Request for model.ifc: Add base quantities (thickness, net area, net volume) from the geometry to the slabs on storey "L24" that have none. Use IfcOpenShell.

First a look at what the model holds.

```python
import ifcopenshell
import ifcopenshell.util.element
import ifcopenshell.util.unit

model = ifcopenshell.open("model.ifc")
print(model.schema)
for unit_type in ("LENGTHUNIT", "AREAUNIT", "VOLUMEUNIT"):
    print(unit_type, ifcopenshell.util.unit.calculate_unit_scale(model, unit_type))
storey = next(s for s in model.by_type("IfcBuildingStorey") if s.Name == "L24")
slabs = [e for e in ifcopenshell.util.element.get_decomposition(storey) if e.is_a("IfcSlab")]
for e in sorted(slabs, key=lambda e: e.id()):
    print(e.id(), e.is_a(), e.Name, list(ifcopenshell.util.element.get_psets(e, qtos_only=True)), sep=" | ")
```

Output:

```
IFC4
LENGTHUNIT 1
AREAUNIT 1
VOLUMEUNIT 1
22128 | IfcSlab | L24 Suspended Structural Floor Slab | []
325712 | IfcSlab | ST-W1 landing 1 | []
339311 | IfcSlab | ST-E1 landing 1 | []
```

```python
import ifcopenshell
import ifcopenshell.api.pset
import ifcopenshell.geom
import ifcopenshell.util.element
import ifcopenshell.util.shape
import ifcopenshell.util.unit

model = ifcopenshell.open("model.ifc")
unit_scale = ifcopenshell.util.unit.calculate_unit_scale(model)
area_scale = ifcopenshell.util.unit.calculate_unit_scale(model, "AREAUNIT")
volume_scale = ifcopenshell.util.unit.calculate_unit_scale(model, "VOLUMEUNIT")
settings = ifcopenshell.geom.settings()

storey = next(s for s in model.by_type("IfcBuildingStorey") if s.Name == "L24")
slabs = [e for e in ifcopenshell.util.element.get_decomposition(storey) if e.is_a("IfcSlab")]

for e in sorted(slabs, key=lambda e: e.id()):
    if ifcopenshell.util.element.get_psets(e, qtos_only=True, should_inherit=False):
        continue
    # Geometry comes back in metres, in the element's own axes.
    shape = ifcopenshell.geom.create_shape(settings, e)
    values = {
        "Width": ifcopenshell.util.shape.get_z(shape.geometry) / unit_scale,
        "NetArea": ifcopenshell.util.shape.get_footprint_area(shape.geometry) / area_scale,
        "NetVolume": ifcopenshell.util.shape.get_volume(shape.geometry) / volume_scale,
    }
    qto = ifcopenshell.api.pset.add_qto(model, product=e, name="Qto_SlabBaseQuantities")
    ifcopenshell.api.pset.edit_qto(model, qto=qto, properties=values)
    print(e.id(), {k: round(v, 3) for k, v in values.items()})

model.write("model-out.ifc")
```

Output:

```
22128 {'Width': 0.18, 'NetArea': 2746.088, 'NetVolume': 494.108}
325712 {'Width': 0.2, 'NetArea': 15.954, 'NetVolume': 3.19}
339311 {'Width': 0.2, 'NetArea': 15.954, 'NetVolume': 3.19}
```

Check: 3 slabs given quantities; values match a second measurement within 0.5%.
